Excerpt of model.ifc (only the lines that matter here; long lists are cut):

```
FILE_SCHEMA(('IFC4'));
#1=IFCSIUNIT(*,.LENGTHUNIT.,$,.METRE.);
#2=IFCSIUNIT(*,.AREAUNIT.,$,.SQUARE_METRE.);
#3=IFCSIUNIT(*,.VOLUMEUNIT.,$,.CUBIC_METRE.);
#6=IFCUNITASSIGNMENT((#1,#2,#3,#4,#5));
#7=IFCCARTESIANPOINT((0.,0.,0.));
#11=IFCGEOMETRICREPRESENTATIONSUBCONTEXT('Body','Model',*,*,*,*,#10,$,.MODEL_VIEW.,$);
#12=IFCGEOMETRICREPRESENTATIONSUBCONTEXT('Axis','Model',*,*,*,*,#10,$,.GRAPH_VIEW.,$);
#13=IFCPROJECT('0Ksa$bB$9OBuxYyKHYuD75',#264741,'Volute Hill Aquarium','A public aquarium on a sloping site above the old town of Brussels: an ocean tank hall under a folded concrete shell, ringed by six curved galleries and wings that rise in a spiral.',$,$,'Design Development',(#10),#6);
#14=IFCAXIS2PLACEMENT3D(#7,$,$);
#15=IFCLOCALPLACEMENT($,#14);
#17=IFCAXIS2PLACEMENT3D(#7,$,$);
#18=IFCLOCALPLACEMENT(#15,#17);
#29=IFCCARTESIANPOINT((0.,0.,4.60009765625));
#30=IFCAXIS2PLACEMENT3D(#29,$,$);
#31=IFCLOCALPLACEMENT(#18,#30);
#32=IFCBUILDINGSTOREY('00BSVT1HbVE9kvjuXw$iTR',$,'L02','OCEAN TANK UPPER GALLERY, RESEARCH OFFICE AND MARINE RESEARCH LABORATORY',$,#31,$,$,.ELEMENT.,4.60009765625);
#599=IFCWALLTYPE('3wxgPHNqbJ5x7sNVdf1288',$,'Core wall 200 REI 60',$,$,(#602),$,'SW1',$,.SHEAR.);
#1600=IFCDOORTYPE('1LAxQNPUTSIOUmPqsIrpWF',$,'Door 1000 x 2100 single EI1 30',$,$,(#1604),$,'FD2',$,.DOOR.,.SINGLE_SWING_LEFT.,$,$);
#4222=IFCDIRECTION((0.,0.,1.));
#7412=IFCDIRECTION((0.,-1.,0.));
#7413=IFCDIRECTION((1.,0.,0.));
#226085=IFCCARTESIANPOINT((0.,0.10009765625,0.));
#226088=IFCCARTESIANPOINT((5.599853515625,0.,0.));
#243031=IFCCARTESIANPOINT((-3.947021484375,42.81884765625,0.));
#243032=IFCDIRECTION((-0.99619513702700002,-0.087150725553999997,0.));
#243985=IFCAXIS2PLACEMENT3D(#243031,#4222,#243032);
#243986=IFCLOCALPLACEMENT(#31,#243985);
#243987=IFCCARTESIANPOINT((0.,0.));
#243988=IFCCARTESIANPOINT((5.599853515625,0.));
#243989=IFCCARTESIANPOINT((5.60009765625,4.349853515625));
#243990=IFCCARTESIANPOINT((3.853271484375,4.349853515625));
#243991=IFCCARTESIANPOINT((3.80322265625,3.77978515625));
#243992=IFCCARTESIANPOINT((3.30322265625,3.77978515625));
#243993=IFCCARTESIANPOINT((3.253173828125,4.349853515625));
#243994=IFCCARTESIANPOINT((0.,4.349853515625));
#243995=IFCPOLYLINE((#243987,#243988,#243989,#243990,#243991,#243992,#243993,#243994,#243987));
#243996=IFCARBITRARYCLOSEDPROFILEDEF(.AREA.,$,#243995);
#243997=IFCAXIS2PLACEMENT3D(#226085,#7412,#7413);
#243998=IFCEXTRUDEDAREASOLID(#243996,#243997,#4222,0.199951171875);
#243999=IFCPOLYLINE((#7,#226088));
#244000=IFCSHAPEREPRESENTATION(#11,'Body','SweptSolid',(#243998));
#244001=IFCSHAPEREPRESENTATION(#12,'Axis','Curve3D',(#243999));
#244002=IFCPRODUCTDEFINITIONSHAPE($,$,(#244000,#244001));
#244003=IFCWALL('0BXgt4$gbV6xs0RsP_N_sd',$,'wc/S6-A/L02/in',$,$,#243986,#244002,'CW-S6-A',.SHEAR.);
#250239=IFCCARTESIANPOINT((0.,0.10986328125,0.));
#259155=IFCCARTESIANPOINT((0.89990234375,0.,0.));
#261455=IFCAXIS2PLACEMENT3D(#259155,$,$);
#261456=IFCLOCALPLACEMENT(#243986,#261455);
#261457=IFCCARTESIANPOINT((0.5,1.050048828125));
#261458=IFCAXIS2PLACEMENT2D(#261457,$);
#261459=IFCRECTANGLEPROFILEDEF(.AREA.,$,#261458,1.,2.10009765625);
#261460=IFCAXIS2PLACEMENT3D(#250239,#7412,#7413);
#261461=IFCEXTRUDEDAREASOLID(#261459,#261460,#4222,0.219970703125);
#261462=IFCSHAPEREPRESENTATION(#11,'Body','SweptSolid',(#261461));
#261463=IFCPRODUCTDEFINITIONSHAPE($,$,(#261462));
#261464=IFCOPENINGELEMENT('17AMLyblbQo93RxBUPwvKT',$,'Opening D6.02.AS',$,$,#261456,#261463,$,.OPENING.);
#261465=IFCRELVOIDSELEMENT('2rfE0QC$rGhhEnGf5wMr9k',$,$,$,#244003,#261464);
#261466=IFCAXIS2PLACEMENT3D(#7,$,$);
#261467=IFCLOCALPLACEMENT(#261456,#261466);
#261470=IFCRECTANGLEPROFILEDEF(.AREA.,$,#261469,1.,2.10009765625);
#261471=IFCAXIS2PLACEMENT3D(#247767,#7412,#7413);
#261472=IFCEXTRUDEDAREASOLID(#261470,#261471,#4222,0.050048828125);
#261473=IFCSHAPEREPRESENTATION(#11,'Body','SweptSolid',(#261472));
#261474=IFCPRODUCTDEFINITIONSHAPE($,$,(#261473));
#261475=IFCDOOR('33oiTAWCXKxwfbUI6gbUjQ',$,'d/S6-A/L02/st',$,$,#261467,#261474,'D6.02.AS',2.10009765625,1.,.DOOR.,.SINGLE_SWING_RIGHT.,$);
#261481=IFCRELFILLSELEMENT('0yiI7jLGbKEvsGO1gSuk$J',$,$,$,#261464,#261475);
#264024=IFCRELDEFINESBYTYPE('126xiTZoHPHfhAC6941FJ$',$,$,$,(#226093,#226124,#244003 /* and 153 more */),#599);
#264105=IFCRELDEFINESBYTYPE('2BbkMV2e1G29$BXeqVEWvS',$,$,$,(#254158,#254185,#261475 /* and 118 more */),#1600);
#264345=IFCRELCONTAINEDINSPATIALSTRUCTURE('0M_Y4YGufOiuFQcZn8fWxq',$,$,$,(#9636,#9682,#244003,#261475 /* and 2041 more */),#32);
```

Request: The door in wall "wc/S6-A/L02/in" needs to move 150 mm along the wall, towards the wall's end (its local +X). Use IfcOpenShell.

```python
import ifcopenshell
import ifcopenshell.api.geometry
import ifcopenshell.util.placement
import ifcopenshell.util.unit

model = ifcopenshell.open("model.ifc")
unit_scale = ifcopenshell.util.unit.calculate_unit_scale(model)

door = model.by_guid("33oiTAWCXKxwfbUI6gbUjQ")
opening = door.FillsVoids[0].RelatingOpeningElement
wall = opening.VoidsElements[0].RelatingBuildingElement

wall_matrix = ifcopenshell.util.placement.get_local_placement(wall.ObjectPlacement)
shift = wall_matrix[:3, 0] * 0.15 / unit_scale
before = ifcopenshell.util.placement.get_local_placement(door.ObjectPlacement)[:3, 3].copy()

# The door is placed relative to its opening, so it follows when the opening moves.
matrix = ifcopenshell.util.placement.get_local_placement(opening.ObjectPlacement)
matrix[:3, 3] += shift
ifcopenshell.api.geometry.edit_object_placement(
    model, product=opening, matrix=matrix, is_si=False, should_transform_children=True
)

after = ifcopenshell.util.placement.get_local_placement(door.ObjectPlacement)[:3, 3]
print("door moved by", (after - before).round(3) + 0.0)

model.write("model_updated.ifc")
```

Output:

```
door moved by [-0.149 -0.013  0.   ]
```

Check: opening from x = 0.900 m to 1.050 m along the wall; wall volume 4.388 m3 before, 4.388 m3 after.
